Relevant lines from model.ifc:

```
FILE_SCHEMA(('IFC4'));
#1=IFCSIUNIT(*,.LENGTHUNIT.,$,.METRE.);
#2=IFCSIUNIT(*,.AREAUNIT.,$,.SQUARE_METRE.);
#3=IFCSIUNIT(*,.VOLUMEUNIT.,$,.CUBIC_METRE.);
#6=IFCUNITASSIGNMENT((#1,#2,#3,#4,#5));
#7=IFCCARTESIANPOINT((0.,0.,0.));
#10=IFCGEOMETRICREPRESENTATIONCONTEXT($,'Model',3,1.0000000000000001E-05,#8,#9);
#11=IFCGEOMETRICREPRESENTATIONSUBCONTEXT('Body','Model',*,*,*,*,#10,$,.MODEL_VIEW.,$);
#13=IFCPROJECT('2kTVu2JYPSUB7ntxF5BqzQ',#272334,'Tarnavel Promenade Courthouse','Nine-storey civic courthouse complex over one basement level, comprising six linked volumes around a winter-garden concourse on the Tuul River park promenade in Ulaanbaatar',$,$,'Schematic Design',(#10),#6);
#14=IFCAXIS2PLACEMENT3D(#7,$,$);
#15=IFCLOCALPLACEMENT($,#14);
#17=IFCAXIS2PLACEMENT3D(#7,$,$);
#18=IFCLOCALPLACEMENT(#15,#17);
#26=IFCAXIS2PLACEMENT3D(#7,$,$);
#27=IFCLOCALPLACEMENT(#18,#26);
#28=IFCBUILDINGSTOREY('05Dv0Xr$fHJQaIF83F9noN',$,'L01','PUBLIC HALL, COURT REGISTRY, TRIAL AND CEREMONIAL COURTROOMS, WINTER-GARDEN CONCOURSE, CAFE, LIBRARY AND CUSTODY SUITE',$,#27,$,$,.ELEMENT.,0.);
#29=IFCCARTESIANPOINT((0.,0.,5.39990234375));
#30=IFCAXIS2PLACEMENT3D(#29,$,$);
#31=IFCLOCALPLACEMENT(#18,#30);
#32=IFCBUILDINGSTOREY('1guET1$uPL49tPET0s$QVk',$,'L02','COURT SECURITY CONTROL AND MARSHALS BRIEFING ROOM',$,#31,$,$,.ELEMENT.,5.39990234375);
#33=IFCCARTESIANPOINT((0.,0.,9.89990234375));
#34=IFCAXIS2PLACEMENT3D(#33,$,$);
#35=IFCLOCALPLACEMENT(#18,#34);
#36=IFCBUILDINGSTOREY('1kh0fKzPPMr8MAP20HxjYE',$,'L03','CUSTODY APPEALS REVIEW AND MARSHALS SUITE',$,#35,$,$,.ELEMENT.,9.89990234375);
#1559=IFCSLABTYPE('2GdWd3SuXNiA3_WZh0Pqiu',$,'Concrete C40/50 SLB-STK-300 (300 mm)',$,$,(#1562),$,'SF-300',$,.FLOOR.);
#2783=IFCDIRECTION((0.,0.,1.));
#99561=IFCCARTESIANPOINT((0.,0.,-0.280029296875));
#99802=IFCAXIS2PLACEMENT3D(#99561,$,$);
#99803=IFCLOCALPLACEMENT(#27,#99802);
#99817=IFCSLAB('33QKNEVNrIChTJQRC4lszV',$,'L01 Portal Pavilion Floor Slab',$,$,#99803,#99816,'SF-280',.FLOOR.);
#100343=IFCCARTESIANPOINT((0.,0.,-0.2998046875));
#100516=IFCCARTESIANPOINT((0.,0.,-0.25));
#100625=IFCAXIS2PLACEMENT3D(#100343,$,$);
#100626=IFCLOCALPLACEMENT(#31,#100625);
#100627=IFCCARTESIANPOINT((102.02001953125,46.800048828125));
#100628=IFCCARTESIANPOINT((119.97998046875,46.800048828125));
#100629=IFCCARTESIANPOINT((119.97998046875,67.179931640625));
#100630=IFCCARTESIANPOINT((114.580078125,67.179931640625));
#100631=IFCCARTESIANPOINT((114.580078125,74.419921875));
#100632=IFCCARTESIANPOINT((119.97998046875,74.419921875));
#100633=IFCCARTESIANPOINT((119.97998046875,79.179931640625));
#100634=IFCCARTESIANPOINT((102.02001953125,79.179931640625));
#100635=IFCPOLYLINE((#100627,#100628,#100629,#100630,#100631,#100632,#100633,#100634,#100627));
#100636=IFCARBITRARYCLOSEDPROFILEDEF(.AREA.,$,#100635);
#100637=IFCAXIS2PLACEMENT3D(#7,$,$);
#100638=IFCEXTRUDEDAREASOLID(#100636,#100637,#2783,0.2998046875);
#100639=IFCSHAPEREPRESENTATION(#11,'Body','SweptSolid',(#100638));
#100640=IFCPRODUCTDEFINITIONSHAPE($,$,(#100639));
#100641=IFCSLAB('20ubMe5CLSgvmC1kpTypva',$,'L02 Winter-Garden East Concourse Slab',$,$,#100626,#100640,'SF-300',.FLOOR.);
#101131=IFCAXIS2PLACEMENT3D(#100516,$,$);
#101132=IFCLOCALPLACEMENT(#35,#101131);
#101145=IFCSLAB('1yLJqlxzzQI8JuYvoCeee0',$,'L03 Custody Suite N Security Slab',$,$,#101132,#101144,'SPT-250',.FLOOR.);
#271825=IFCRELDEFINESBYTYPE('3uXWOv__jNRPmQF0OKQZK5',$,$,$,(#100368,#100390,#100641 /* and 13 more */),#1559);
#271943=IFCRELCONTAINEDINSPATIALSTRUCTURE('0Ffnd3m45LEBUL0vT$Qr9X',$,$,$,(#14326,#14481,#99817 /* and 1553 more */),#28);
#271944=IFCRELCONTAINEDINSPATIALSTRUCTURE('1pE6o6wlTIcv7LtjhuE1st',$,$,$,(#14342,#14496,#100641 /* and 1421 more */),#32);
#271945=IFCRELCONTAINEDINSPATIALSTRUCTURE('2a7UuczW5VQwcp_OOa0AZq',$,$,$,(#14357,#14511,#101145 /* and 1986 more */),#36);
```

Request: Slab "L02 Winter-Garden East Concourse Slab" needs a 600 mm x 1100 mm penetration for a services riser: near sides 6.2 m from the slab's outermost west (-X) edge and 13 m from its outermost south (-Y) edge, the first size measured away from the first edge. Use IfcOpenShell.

```python
import numpy as np
import ifcopenshell
import ifcopenshell.api.feature
import ifcopenshell.api.geometry
import ifcopenshell.api.root
import ifcopenshell.geom
import ifcopenshell.util.placement
import ifcopenshell.util.representation
import ifcopenshell.util.shape
import ifcopenshell.util.unit

model = ifcopenshell.open("model.ifc")
unit_scale = ifcopenshell.util.unit.calculate_unit_scale(model)
settings = ifcopenshell.geom.settings()


def volume(element):
    """Net volume in cubic metres, openings subtracted."""
    shape = ifcopenshell.geom.create_shape(settings, element)
    return ifcopenshell.util.shape.get_volume(shape.geometry)


slab = model.by_id(100641)
before = volume(slab)

# Extent in the slab's own axes, in metres. The edges named are its -X and -Y sides.
slab_shape = ifcopenshell.geom.create_shape(settings, slab)
vertices = ifcopenshell.util.shape.get_vertices(slab_shape.geometry)
x_min, y_min, bottom = vertices.min(axis=0)
top = vertices[:, 2].max()

opening = ifcopenshell.api.root.create_entity(model, ifc_class="IfcOpeningElement", name="Services riser opening", predefined_type="OPENING")
context = ifcopenshell.util.representation.get_context(model, "Model", "Body", "MODEL_VIEW")
width, depth = 0.6, 1.1
outline = [(0.0, 0.0), (width, 0.0), (width, depth), (0.0, depth), (0.0, 0.0)]
# Overshoot both faces by 50 mm so the cut is clean.
shape = ifcopenshell.api.geometry.add_slab_representation(
    model, context=context, depth=top - bottom + 0.1, polyline=outline
)
ifcopenshell.api.geometry.assign_representation(model, product=opening, representation=shape)

matrix = ifcopenshell.util.placement.get_local_placement(slab.ObjectPlacement)
matrix[:, 3] = matrix @ np.append(np.array([x_min + 6.2, y_min + 13, bottom - 0.05]) / unit_scale, 1.0)
ifcopenshell.api.geometry.edit_object_placement(model, product=opening, matrix=matrix, is_si=False)
ifcopenshell.api.feature.add_feature(model, feature=opening, element=slab)

after = volume(slab)

print(f"slab volume {before:.3f} -> {after:.3f} m3")

model.write("model_edited.ifc")
```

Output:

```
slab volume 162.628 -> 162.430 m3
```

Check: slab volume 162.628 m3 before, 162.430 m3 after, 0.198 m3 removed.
